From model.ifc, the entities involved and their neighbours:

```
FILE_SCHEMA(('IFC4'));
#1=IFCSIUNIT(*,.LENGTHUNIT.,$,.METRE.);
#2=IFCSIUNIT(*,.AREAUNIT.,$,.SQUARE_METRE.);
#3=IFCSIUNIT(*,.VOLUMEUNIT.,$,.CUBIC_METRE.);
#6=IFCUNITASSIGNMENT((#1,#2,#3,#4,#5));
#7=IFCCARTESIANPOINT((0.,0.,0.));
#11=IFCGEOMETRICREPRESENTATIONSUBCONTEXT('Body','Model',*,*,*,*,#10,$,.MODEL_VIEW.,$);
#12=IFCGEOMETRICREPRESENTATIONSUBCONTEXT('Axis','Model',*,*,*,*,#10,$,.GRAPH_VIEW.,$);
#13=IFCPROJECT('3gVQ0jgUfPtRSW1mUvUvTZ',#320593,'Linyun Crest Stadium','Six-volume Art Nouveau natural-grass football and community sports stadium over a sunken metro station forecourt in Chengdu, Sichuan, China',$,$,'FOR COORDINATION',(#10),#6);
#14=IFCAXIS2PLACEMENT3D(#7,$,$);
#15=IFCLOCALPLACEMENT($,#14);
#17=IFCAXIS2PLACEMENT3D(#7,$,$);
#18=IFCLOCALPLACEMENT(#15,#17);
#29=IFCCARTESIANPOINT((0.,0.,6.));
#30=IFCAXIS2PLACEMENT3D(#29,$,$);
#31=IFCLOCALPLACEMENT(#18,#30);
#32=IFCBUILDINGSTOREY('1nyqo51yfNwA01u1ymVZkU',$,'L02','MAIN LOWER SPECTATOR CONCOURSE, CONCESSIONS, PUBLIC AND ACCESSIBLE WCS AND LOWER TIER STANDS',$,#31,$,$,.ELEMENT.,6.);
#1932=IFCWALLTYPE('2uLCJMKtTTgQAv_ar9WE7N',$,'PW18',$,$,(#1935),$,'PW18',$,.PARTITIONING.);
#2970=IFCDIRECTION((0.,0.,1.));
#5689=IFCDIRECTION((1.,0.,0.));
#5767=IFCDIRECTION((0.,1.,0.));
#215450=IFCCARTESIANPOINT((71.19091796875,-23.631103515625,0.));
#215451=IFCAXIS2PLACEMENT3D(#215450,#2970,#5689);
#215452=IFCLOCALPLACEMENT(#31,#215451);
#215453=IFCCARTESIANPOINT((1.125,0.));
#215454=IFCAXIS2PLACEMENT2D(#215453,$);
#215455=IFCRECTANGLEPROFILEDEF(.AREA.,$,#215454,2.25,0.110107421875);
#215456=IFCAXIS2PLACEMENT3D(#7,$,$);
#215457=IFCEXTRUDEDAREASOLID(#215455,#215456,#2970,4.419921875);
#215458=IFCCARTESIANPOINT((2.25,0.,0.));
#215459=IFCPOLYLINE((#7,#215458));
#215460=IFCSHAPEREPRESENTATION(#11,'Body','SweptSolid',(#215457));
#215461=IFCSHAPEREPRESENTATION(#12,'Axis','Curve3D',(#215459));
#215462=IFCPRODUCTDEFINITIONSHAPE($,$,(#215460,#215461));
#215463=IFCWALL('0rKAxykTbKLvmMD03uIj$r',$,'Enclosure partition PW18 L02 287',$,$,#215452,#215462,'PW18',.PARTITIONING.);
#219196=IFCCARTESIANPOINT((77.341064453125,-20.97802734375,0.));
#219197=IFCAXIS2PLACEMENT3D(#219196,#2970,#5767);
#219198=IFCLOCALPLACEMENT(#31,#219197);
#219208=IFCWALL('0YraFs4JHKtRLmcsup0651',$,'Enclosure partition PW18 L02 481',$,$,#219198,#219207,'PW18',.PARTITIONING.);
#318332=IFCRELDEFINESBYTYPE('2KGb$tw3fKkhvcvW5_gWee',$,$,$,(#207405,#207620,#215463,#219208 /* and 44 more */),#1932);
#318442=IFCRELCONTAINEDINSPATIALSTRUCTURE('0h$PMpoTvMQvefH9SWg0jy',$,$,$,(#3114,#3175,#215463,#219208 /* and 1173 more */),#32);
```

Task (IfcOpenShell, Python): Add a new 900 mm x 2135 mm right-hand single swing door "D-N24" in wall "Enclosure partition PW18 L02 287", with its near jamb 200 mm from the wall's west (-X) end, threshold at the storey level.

```python
import numpy as np
import ifcopenshell
import ifcopenshell.api.feature
import ifcopenshell.api.geometry
import ifcopenshell.api.root
import ifcopenshell.api.spatial
import ifcopenshell.geom
import ifcopenshell.util.element
import ifcopenshell.util.placement
import ifcopenshell.util.representation
import ifcopenshell.util.shape
import ifcopenshell.util.unit

model = ifcopenshell.open("model.ifc")
unit_scale = ifcopenshell.util.unit.calculate_unit_scale(model)
settings = ifcopenshell.geom.settings()


def volume(element):
    """Net volume in cubic metres, openings subtracted."""
    shape = ifcopenshell.geom.create_shape(settings, element)
    return ifcopenshell.util.shape.get_volume(shape.geometry)


wall = model.by_guid("0rKAxykTbKLvmMD03uIj$r")
storey = ifcopenshell.util.element.get_container(wall, ifc_class="IfcBuildingStorey")
context = ifcopenshell.util.representation.get_context(model, "Model", "Body", "MODEL_VIEW")
before = volume(wall)

width, height, from_end, sill = 0.9, 2.135, 0.2, 0.0  # metres

# The wall runs along its own X axis, and the end named is its -X end.
wall_shape = ifcopenshell.geom.create_shape(settings, wall)
x, y, z = ifcopenshell.util.shape.get_vertices(wall_shape.geometry).T
start = x.min() + from_end
face, thickness = float(y.min()), float(y.max() - y.min())
wall_matrix = ifcopenshell.util.placement.get_local_placement(wall.ObjectPlacement)
level = ifcopenshell.util.placement.get_local_placement(storey.ObjectPlacement)[2, 3]


def in_wall(x, y):
    """Placement at x, y metres in the wall's axes, at sill height."""
    matrix = wall_matrix.copy()
    matrix[:, 3] = wall_matrix @ np.array([x / unit_scale, y / unit_scale, 0.0, 1.0])
    matrix[2, 3] = level + sill / unit_scale
    return matrix


# Opening: a box that overshoots both wall faces by 50 mm.
opening = ifcopenshell.api.root.create_entity(model, ifc_class="IfcOpeningElement", predefined_type="OPENING")
box = ifcopenshell.api.geometry.add_wall_representation(
    model, context=context, length=width, height=height, thickness=thickness + 0.1
)
ifcopenshell.api.geometry.assign_representation(model, product=opening, representation=box)
ifcopenshell.api.geometry.edit_object_placement(model, product=opening, matrix=in_wall(start, face - 0.05), is_si=False)
ifcopenshell.api.feature.add_feature(model, feature=opening, element=wall)

door = ifcopenshell.api.root.create_entity(model, ifc_class="IfcDoor", name="D-N24", predefined_type="DOOR")
door.OverallWidth, door.OverallHeight = width / unit_scale, height / unit_scale
door.OperationType = "SINGLE_SWING_RIGHT"
body = ifcopenshell.api.geometry.add_door_representation(
    model,
    context=context,
    overall_width=door.OverallWidth,
    overall_height=door.OverallHeight,
    operation_type="SINGLE_SWING_RIGHT",
    lining_properties={"LiningDepth": thickness / unit_scale, "ThresholdDepth": thickness / unit_scale},
)
ifcopenshell.api.geometry.assign_representation(model, product=door, representation=body)
ifcopenshell.api.spatial.assign_container(model, products=[door], relating_structure=storey)
ifcopenshell.api.feature.add_filling(model, opening=opening, element=door)

# The lining spans the wall, so the door starts at the wall face.
ifcopenshell.api.geometry.edit_object_placement(model, product=door, matrix=in_wall(start, face), is_si=False)

after = volume(wall)

print(f"wall volume {before:.3f} -> {after:.3f} m3")

model.write("model_updated.ifc")
```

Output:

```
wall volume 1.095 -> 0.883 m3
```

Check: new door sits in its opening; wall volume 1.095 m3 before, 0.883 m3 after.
